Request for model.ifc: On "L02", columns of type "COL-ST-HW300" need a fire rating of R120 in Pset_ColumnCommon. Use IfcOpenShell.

First a look at what the model holds.

```python
import ifcopenshell
import ifcopenshell.util.element

model = ifcopenshell.open("model.ifc")
print(model.schema)
storey = next(s for s in model.by_type("IfcBuildingStorey") if s.Name == "L02")
columns = [e for e in ifcopenshell.util.element.get_decomposition(storey) if e.is_a("IfcColumn")]
seen = {}
for e in columns:
    element_type = ifcopenshell.util.element.get_type(e)
    key = (element_type.Name if element_type != e and element_type else None, ifcopenshell.util.element.get_pset(e, "Pset_ColumnCommon", "FireRating"))
    seen[key] = seen.get(key, 0) + 1
for (name, value), count in sorted(seen.items(), key=str):
    print(count, "x", name, "|", value)
```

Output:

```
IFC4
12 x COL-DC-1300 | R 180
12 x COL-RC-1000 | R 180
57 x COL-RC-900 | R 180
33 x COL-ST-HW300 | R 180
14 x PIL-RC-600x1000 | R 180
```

```python
import ifcopenshell
import ifcopenshell.api.pset
import ifcopenshell.util.element

model = ifcopenshell.open("model.ifc")

storey = next(s for s in model.by_type("IfcBuildingStorey") if s.Name == "L02")
columns = [e for e in ifcopenshell.util.element.get_decomposition(storey) if e.is_a("IfcColumn")]

count = 0
for e in columns:
    element_type = ifcopenshell.util.element.get_type(e)
    if element_type in (None, e) or element_type.Name != "COL-ST-HW300":
        continue
    # add_pset returns the element's existing set when there is one.
    pset = ifcopenshell.api.pset.add_pset(model, product=e, name="Pset_ColumnCommon")
    ifcopenshell.api.pset.edit_pset(model, pset=pset, properties={"FireRating": "R120"})
    count += 1

print(count, "columns updated")

model.write("model-out.ifc")
```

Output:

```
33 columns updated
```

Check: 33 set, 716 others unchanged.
